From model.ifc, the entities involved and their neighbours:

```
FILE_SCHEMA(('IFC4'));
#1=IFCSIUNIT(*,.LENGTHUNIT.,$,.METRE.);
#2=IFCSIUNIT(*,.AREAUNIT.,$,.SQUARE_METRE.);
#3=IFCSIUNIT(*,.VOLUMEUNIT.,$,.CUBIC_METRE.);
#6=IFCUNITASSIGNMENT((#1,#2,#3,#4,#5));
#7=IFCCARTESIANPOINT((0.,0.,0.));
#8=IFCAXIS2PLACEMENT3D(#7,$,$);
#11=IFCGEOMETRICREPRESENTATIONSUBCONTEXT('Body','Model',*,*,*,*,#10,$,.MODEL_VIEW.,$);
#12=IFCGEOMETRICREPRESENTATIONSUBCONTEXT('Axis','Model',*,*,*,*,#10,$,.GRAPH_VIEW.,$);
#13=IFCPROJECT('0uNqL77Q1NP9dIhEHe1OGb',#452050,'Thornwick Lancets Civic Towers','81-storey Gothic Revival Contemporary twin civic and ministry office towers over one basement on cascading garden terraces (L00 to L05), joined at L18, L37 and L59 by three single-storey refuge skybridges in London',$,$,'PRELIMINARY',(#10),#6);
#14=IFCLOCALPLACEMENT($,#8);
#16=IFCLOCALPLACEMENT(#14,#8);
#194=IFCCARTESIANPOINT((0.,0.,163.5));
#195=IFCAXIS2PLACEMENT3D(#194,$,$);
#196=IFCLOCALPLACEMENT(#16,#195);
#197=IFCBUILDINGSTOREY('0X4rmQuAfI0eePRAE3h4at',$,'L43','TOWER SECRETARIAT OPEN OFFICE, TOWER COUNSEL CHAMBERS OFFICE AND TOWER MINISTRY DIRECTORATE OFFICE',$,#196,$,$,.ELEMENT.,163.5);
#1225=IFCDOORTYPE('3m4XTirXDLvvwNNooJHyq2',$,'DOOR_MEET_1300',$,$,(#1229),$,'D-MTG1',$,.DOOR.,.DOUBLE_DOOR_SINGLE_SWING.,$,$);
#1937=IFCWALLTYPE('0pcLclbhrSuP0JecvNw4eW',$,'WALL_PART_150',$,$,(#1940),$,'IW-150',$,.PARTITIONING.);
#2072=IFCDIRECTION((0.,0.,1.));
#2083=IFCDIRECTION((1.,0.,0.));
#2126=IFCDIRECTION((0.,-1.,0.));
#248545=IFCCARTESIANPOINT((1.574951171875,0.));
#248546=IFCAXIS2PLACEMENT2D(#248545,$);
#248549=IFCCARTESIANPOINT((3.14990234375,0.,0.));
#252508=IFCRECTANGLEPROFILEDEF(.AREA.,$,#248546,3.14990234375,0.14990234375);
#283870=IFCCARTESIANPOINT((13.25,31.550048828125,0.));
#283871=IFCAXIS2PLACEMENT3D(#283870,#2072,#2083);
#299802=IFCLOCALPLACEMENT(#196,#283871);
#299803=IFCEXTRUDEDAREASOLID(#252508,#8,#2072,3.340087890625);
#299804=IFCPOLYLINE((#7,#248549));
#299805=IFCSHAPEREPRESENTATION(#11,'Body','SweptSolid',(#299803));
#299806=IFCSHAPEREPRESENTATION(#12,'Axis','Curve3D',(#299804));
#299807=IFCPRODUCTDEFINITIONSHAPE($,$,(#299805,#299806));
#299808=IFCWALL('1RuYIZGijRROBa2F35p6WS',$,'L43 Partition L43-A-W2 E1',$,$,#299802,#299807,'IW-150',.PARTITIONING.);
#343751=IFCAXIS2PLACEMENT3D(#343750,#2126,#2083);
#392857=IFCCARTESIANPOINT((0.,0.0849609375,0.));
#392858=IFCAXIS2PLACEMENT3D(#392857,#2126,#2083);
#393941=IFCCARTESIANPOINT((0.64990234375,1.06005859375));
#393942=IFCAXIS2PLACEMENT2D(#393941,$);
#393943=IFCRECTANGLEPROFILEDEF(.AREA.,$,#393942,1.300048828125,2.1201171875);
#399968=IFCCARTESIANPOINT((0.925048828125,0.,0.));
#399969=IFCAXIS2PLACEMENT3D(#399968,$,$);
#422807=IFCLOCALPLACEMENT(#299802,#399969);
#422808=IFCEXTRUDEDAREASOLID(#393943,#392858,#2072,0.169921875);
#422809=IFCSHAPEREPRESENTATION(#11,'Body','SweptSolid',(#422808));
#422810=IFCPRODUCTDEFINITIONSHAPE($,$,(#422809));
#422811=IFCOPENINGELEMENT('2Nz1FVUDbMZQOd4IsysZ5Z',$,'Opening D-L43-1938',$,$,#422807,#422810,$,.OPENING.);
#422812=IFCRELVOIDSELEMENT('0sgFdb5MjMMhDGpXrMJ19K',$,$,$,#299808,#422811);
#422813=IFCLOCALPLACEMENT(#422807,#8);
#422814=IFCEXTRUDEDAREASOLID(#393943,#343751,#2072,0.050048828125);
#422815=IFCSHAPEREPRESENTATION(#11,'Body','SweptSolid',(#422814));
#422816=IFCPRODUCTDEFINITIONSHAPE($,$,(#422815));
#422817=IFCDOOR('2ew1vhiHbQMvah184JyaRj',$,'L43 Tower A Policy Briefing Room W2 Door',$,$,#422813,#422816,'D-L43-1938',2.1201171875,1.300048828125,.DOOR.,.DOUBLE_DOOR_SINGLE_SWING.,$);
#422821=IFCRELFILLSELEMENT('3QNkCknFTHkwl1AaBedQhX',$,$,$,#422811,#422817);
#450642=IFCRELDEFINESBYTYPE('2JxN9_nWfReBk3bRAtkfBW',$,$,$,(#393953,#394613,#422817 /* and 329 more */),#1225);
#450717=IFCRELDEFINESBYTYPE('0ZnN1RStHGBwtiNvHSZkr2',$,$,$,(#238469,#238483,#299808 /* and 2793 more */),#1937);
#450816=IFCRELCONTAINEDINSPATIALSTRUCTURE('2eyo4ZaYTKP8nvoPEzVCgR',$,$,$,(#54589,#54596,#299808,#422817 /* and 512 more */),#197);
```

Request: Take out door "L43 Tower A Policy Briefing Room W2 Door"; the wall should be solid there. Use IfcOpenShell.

```python
import ifcopenshell
import ifcopenshell.api.feature
import ifcopenshell.api.root
import ifcopenshell.geom
import ifcopenshell.util.shape

model = ifcopenshell.open("model.ifc")
settings = ifcopenshell.geom.settings()


def volume(element):
    """Net volume in cubic metres, openings subtracted."""
    shape = ifcopenshell.geom.create_shape(settings, element)
    return ifcopenshell.util.shape.get_volume(shape.geometry)


door = model.by_guid("2ew1vhiHbQMvah184JyaRj")
opening = door.FillsVoids[0].RelatingOpeningElement
wall = opening.VoidsElements[0].RelatingBuildingElement
before = volume(wall)

ifcopenshell.api.root.remove_product(model, product=door)
ifcopenshell.api.feature.remove_feature(model, feature=opening)

after = volume(wall)

print(f"wall volume {before:.3f} -> {after:.3f} m3")

model.write("model_rev.ifc")
```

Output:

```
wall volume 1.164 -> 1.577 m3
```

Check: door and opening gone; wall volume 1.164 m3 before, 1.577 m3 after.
